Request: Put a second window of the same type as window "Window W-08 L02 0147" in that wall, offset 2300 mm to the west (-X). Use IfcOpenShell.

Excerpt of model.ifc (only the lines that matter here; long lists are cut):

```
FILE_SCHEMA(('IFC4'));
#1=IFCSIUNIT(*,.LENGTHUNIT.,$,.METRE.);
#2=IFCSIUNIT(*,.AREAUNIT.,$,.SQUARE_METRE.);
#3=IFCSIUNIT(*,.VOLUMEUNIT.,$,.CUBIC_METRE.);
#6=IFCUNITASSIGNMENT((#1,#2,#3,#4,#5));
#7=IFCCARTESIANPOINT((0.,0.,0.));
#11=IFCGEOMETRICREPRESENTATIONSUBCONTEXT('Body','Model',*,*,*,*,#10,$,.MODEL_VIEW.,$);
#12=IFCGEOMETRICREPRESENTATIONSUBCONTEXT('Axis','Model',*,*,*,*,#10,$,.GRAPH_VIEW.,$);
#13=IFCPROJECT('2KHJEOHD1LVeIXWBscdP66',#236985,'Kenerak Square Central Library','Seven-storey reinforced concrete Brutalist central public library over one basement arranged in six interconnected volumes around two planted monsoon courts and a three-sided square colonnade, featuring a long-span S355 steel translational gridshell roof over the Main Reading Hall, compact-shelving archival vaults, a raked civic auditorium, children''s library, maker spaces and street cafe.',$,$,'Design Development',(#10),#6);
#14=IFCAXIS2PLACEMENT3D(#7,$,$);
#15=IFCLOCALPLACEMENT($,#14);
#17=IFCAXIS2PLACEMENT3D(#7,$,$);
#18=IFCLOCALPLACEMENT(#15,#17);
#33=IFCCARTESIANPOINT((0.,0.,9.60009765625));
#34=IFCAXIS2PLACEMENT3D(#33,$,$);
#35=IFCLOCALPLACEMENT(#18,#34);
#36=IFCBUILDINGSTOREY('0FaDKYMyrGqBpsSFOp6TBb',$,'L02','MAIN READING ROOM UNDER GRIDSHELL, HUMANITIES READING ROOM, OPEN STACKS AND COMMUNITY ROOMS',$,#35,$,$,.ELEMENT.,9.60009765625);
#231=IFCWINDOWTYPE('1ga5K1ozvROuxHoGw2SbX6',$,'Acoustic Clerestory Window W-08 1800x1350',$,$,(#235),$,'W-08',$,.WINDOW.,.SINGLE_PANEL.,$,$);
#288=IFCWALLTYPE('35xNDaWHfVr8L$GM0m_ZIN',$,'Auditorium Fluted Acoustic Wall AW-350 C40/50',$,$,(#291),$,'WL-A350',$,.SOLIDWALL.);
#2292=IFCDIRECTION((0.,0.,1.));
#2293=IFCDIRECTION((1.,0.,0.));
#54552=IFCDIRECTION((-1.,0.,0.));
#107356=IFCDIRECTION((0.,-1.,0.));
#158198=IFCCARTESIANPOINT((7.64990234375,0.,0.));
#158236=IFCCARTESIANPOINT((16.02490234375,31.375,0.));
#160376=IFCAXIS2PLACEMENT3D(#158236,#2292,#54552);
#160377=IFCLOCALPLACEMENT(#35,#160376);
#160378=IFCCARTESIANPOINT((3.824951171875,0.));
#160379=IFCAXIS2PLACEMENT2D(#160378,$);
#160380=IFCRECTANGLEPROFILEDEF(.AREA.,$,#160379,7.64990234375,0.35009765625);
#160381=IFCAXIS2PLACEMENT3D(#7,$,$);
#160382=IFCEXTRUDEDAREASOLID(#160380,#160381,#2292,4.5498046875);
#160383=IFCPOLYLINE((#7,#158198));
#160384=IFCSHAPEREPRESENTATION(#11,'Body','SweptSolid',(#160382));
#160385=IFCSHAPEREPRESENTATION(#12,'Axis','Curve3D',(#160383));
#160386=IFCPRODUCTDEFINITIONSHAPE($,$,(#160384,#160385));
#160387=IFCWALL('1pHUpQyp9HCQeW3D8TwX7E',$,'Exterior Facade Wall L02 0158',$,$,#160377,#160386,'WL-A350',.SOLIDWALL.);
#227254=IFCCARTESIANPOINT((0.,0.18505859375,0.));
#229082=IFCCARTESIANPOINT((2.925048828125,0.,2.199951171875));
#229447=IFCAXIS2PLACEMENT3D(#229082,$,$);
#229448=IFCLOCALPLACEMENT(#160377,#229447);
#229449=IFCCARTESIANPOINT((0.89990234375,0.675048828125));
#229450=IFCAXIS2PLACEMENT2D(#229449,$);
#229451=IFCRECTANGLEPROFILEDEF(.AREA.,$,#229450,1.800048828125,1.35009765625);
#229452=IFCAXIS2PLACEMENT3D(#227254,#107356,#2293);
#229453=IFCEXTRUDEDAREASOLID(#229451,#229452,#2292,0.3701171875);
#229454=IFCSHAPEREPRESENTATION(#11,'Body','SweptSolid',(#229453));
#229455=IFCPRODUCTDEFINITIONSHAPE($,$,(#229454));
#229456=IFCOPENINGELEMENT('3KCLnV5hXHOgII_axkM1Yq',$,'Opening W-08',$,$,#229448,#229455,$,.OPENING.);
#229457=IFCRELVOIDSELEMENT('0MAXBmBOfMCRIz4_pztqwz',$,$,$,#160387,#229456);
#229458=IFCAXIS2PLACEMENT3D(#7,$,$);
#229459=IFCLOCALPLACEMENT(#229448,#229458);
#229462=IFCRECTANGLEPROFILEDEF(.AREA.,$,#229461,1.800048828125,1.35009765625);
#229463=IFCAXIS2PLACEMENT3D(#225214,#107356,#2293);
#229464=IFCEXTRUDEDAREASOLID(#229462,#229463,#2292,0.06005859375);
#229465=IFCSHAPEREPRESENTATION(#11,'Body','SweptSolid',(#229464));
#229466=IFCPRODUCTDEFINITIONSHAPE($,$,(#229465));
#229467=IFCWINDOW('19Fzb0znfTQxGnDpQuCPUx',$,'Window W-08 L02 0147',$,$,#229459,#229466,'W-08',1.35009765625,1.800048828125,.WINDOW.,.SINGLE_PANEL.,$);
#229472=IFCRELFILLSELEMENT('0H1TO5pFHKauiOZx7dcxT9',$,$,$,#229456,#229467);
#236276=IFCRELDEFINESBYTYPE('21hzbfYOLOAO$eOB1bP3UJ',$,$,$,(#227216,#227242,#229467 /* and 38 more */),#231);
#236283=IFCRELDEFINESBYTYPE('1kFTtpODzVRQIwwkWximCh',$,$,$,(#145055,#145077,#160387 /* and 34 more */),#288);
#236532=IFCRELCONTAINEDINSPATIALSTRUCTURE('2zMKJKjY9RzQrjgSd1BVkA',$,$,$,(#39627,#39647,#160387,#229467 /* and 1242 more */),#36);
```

```python
import ifcopenshell
import ifcopenshell.api.feature
import ifcopenshell.api.geometry
import ifcopenshell.api.root
import ifcopenshell.geom
import ifcopenshell.util.element
import ifcopenshell.util.placement
import ifcopenshell.util.shape
import ifcopenshell.util.unit

model = ifcopenshell.open("model.ifc")
unit_scale = ifcopenshell.util.unit.calculate_unit_scale(model)
settings = ifcopenshell.geom.settings()


def volume(element):
    """Net volume in cubic metres, openings subtracted."""
    shape = ifcopenshell.geom.create_shape(settings, element)
    return ifcopenshell.util.shape.get_volume(shape.geometry)


window = model.by_guid("19Fzb0znfTQxGnDpQuCPUx")
opening = window.FillsVoids[0].RelatingOpeningElement
wall = opening.VoidsElements[0].RelatingBuildingElement
before = volume(wall)
shift = ifcopenshell.util.placement.get_local_placement(wall.ObjectPlacement)[:3, 0] * 2.3 / unit_scale

# copy_class copies the void relationship, type, container and properties, but no geometry.
new_opening = ifcopenshell.api.root.copy_class(model, product=opening)
new_opening.Representation = ifcopenshell.util.element.copy_deep(
    model, opening.Representation, exclude=["IfcGeometricRepresentationContext", "IfcRepresentationMap"]
)
new_window = ifcopenshell.api.root.copy_class(model, product=window)
new_window.Representation = ifcopenshell.util.element.copy_deep(
    model, window.Representation, exclude=["IfcGeometricRepresentationContext", "IfcRepresentationMap"]
)
new_window.Tag = None
ifcopenshell.api.feature.add_filling(model, opening=new_opening, element=new_window)

for old, new in ((opening, new_opening), (window, new_window)):
    matrix = ifcopenshell.util.placement.get_local_placement(old.ObjectPlacement)
    matrix[:3, 3] += shift
    ifcopenshell.api.geometry.edit_object_placement(model, product=new, matrix=matrix, is_si=False)

after = volume(wall)

print(f"wall volume {before:.3f} -> {after:.3f} m3")

model.write("model_rev.ifc")
```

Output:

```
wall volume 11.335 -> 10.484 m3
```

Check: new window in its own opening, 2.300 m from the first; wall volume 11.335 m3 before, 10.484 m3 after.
